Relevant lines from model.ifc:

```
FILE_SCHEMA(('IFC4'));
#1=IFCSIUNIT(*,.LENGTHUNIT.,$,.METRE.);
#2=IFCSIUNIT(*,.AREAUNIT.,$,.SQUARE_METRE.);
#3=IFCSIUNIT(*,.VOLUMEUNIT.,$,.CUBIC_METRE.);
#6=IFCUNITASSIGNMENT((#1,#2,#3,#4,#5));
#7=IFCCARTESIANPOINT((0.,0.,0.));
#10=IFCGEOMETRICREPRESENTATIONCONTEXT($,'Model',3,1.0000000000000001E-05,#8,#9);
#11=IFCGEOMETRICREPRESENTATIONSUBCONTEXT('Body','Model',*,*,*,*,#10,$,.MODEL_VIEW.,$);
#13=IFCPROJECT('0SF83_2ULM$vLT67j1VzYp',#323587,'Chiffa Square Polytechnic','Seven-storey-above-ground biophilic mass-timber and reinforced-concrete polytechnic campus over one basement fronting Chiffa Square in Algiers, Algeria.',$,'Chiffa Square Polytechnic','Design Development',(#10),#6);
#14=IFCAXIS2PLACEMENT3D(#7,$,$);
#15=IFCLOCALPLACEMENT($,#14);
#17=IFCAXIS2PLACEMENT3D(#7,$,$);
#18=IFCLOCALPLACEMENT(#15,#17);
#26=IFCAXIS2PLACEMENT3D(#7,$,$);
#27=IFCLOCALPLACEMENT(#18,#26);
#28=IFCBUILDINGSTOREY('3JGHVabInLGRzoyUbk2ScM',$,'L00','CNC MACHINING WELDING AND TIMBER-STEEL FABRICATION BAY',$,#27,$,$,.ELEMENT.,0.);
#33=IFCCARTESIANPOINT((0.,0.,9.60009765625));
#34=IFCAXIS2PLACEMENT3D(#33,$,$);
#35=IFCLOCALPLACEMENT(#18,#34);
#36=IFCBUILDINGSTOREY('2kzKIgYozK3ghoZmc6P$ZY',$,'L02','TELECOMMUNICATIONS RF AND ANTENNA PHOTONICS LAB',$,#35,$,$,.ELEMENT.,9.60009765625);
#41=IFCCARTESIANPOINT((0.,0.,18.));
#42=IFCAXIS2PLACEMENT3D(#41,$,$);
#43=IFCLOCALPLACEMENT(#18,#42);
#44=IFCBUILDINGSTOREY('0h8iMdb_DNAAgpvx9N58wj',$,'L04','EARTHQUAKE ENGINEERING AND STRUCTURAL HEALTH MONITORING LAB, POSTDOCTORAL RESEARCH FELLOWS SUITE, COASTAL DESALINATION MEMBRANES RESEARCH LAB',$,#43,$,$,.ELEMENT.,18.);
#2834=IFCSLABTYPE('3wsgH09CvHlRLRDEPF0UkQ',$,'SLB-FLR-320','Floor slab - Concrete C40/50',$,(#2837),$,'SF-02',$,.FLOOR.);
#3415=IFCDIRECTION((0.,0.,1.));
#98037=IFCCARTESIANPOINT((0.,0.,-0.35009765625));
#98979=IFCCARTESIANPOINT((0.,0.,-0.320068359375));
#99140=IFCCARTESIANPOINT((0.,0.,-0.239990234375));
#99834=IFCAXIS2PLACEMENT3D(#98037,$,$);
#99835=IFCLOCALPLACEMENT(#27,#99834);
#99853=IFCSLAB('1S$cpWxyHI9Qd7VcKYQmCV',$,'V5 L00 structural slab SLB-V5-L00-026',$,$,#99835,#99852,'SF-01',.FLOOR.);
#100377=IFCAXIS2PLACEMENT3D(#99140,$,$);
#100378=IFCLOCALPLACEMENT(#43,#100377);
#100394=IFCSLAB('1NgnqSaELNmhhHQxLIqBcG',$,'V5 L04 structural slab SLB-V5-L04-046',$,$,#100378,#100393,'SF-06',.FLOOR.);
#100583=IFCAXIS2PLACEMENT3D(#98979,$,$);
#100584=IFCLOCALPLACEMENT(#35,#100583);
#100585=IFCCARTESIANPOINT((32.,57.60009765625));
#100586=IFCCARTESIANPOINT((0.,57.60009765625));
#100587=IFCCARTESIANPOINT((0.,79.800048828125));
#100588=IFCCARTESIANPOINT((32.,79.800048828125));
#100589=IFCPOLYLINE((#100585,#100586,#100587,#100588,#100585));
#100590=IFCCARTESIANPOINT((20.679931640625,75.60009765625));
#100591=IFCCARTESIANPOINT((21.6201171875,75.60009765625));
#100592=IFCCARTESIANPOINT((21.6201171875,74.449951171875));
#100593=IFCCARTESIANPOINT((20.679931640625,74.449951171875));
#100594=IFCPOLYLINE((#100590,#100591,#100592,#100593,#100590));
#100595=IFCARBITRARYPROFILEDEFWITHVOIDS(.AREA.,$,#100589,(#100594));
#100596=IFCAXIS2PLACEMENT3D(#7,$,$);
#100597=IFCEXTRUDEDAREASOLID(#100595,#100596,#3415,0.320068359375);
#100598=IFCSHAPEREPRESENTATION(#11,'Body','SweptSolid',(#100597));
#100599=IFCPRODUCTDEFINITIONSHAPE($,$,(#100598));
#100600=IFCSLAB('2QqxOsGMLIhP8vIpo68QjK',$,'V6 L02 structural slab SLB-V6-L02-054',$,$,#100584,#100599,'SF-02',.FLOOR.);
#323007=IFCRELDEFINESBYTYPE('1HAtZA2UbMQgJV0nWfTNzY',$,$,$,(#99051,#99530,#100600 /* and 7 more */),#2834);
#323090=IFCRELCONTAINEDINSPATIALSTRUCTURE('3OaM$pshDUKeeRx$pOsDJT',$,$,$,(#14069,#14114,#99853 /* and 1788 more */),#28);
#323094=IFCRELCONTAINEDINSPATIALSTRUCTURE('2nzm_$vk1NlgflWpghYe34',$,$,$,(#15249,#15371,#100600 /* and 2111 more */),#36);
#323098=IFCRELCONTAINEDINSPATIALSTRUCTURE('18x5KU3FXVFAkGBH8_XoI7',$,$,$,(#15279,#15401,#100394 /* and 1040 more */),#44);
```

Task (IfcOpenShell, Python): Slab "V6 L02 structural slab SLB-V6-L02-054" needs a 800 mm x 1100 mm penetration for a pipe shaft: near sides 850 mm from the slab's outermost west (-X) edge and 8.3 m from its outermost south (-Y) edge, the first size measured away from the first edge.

```python
import numpy as np
import ifcopenshell
import ifcopenshell.api.feature
import ifcopenshell.api.geometry
import ifcopenshell.api.root
import ifcopenshell.geom
import ifcopenshell.util.placement
import ifcopenshell.util.representation
import ifcopenshell.util.shape
import ifcopenshell.util.unit

model = ifcopenshell.open("model.ifc")
unit_scale = ifcopenshell.util.unit.calculate_unit_scale(model)
settings = ifcopenshell.geom.settings()


def volume(element):
    """Net volume in cubic metres, openings subtracted."""
    shape = ifcopenshell.geom.create_shape(settings, element)
    return ifcopenshell.util.shape.get_volume(shape.geometry)


slab = model.by_id(100600)
before = volume(slab)

# Extent in the slab's own axes, in metres. The edges named are its -X and -Y sides.
slab_shape = ifcopenshell.geom.create_shape(settings, slab)
vertices = ifcopenshell.util.shape.get_vertices(slab_shape.geometry)
x_min, y_min, bottom = vertices.min(axis=0)
top = vertices[:, 2].max()

opening = ifcopenshell.api.root.create_entity(model, ifc_class="IfcOpeningElement", name="Pipe shaft opening", predefined_type="OPENING")
context = ifcopenshell.util.representation.get_context(model, "Model", "Body", "MODEL_VIEW")
width, depth = 0.8, 1.1
outline = [(0.0, 0.0), (width, 0.0), (width, depth), (0.0, depth), (0.0, 0.0)]
# Overshoot both faces by 50 mm so the cut is clean.
shape = ifcopenshell.api.geometry.add_slab_representation(
    model, context=context, depth=top - bottom + 0.1, polyline=outline
)
ifcopenshell.api.geometry.assign_representation(model, product=opening, representation=shape)

matrix = ifcopenshell.util.placement.get_local_placement(slab.ObjectPlacement)
matrix[:, 3] = matrix @ np.append(np.array([x_min + 0.85, y_min + 8.3, bottom - 0.05]) / unit_scale, 1.0)
ifcopenshell.api.geometry.edit_object_placement(model, product=opening, matrix=matrix, is_si=False)
ifcopenshell.api.feature.add_feature(model, feature=opening, element=slab)

after = volume(slab)

print(f"slab volume {before:.3f} -> {after:.3f} m3")

model.write("model_v2.ifc")
```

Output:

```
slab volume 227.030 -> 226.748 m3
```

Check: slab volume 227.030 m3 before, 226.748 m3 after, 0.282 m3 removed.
